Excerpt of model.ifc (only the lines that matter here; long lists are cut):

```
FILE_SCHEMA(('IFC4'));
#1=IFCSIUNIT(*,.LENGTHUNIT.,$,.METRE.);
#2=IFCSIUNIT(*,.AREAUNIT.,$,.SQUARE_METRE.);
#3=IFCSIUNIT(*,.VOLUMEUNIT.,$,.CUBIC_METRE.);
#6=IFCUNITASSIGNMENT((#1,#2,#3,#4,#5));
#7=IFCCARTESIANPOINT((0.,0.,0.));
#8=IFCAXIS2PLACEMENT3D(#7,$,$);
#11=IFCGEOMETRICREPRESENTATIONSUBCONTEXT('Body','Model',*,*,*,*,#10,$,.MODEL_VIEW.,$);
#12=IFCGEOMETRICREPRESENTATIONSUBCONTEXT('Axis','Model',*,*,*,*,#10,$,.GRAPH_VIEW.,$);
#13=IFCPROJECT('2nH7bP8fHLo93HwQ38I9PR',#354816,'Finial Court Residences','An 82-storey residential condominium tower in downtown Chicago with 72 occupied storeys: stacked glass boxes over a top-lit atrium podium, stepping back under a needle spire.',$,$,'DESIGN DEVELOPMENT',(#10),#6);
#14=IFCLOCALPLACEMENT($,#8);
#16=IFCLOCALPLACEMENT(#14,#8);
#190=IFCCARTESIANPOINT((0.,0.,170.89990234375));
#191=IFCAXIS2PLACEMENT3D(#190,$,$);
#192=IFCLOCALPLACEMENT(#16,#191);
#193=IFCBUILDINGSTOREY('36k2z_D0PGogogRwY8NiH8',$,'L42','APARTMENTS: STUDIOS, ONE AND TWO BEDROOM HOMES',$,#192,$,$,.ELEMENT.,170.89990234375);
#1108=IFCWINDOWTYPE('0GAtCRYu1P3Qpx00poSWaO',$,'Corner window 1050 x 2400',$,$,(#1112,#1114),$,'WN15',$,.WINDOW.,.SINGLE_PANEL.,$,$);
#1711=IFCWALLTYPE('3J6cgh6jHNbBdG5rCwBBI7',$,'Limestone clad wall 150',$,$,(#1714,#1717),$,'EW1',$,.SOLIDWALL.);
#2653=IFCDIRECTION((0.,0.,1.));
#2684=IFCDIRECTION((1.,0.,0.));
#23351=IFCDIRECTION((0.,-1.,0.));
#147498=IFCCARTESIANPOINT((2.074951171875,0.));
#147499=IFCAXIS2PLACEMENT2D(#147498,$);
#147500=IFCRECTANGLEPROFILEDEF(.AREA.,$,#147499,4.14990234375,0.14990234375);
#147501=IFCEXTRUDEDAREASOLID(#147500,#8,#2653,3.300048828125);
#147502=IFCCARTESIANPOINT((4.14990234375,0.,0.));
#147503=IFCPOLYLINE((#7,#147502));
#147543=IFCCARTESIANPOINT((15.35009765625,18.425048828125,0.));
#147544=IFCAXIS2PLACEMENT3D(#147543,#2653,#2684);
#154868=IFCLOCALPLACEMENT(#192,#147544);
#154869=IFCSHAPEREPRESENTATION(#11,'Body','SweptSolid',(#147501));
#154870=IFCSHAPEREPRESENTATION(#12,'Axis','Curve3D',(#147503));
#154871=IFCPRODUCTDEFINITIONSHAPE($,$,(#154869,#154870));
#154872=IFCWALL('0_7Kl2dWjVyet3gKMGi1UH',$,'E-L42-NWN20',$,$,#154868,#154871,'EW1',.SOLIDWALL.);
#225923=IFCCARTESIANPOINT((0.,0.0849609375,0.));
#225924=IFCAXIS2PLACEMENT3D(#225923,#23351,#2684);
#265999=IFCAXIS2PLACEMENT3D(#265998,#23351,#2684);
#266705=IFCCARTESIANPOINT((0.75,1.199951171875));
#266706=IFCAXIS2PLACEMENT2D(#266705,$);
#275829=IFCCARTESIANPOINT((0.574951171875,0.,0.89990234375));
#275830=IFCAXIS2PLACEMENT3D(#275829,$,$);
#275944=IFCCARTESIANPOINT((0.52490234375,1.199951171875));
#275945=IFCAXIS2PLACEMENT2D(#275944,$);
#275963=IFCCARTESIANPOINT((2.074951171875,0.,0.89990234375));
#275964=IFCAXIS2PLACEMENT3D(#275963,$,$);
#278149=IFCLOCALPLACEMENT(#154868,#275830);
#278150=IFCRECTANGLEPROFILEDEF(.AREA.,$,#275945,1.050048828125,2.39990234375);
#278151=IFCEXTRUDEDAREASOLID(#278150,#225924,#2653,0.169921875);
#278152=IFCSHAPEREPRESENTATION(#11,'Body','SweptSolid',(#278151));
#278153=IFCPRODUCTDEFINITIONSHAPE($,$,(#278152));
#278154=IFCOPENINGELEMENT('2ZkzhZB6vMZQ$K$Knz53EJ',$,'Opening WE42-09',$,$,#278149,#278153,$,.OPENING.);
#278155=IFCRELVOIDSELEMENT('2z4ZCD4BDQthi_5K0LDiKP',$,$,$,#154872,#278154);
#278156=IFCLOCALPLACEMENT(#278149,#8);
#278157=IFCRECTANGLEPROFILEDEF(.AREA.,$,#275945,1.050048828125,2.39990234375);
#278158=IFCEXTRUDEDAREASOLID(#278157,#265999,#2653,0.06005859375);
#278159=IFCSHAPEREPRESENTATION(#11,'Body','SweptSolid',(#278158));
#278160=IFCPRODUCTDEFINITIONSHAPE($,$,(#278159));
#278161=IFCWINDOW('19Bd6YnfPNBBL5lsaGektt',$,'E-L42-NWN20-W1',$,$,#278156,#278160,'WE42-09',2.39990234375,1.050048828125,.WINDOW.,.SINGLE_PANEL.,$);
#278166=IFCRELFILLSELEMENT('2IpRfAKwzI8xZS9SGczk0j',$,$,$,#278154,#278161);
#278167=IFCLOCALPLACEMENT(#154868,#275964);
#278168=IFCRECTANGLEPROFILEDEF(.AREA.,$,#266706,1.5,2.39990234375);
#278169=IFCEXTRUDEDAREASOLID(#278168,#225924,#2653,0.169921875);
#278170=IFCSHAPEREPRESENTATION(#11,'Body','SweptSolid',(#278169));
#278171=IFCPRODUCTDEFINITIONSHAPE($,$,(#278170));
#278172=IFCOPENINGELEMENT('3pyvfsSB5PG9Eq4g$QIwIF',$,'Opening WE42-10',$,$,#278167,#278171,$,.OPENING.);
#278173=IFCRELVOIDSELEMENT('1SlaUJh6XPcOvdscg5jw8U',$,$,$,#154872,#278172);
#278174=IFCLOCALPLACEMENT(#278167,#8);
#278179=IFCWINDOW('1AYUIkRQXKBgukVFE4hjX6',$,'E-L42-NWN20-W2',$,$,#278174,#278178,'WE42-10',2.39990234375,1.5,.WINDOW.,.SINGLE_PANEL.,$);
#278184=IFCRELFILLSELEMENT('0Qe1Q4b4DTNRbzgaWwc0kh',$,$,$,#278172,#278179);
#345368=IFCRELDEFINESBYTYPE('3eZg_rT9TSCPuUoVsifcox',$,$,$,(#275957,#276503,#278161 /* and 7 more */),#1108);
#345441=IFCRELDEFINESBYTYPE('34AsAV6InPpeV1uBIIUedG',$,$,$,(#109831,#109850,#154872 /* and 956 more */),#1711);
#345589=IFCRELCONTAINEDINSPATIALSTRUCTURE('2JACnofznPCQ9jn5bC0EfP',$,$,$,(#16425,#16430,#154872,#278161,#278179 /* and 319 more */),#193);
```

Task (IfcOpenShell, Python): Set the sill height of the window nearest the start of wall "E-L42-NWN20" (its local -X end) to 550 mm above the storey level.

```python
import numpy as np
import ifcopenshell
import ifcopenshell.api.geometry
import ifcopenshell.geom
import ifcopenshell.util.element
import ifcopenshell.util.placement
import ifcopenshell.util.shape
import ifcopenshell.util.unit

model = ifcopenshell.open("model.ifc")
unit_scale = ifcopenshell.util.unit.calculate_unit_scale(model)

window = model.by_id(278161)
opening = window.FillsVoids[0].RelatingOpeningElement
storey = ifcopenshell.util.element.get_container(window, ifc_class="IfcBuildingStorey")
level = ifcopenshell.util.placement.get_local_placement(storey.ObjectPlacement)[2, 3]

# The opening's origin need not be at the sill, so measure its lowest point.
shape = ifcopenshell.geom.create_shape(ifcopenshell.geom.settings(), opening)
bottom = ifcopenshell.util.shape.get_shape_bottom_elevation(shape, shape.geometry) / unit_scale
dz = level + 0.55 - bottom

shift = np.array([0.0, 0.0, dz])
# The window is placed relative to its opening, so it follows when the opening moves.
matrix = ifcopenshell.util.placement.get_local_placement(opening.ObjectPlacement)
matrix[:3, 3] += shift
ifcopenshell.api.geometry.edit_object_placement(
    model, product=opening, matrix=matrix, is_si=False, should_transform_children=True
)

print(f"moved by {dz * unit_scale:+.3f} m")

model.write("model-out.ifc")
```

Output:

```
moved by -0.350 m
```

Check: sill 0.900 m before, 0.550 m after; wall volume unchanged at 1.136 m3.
